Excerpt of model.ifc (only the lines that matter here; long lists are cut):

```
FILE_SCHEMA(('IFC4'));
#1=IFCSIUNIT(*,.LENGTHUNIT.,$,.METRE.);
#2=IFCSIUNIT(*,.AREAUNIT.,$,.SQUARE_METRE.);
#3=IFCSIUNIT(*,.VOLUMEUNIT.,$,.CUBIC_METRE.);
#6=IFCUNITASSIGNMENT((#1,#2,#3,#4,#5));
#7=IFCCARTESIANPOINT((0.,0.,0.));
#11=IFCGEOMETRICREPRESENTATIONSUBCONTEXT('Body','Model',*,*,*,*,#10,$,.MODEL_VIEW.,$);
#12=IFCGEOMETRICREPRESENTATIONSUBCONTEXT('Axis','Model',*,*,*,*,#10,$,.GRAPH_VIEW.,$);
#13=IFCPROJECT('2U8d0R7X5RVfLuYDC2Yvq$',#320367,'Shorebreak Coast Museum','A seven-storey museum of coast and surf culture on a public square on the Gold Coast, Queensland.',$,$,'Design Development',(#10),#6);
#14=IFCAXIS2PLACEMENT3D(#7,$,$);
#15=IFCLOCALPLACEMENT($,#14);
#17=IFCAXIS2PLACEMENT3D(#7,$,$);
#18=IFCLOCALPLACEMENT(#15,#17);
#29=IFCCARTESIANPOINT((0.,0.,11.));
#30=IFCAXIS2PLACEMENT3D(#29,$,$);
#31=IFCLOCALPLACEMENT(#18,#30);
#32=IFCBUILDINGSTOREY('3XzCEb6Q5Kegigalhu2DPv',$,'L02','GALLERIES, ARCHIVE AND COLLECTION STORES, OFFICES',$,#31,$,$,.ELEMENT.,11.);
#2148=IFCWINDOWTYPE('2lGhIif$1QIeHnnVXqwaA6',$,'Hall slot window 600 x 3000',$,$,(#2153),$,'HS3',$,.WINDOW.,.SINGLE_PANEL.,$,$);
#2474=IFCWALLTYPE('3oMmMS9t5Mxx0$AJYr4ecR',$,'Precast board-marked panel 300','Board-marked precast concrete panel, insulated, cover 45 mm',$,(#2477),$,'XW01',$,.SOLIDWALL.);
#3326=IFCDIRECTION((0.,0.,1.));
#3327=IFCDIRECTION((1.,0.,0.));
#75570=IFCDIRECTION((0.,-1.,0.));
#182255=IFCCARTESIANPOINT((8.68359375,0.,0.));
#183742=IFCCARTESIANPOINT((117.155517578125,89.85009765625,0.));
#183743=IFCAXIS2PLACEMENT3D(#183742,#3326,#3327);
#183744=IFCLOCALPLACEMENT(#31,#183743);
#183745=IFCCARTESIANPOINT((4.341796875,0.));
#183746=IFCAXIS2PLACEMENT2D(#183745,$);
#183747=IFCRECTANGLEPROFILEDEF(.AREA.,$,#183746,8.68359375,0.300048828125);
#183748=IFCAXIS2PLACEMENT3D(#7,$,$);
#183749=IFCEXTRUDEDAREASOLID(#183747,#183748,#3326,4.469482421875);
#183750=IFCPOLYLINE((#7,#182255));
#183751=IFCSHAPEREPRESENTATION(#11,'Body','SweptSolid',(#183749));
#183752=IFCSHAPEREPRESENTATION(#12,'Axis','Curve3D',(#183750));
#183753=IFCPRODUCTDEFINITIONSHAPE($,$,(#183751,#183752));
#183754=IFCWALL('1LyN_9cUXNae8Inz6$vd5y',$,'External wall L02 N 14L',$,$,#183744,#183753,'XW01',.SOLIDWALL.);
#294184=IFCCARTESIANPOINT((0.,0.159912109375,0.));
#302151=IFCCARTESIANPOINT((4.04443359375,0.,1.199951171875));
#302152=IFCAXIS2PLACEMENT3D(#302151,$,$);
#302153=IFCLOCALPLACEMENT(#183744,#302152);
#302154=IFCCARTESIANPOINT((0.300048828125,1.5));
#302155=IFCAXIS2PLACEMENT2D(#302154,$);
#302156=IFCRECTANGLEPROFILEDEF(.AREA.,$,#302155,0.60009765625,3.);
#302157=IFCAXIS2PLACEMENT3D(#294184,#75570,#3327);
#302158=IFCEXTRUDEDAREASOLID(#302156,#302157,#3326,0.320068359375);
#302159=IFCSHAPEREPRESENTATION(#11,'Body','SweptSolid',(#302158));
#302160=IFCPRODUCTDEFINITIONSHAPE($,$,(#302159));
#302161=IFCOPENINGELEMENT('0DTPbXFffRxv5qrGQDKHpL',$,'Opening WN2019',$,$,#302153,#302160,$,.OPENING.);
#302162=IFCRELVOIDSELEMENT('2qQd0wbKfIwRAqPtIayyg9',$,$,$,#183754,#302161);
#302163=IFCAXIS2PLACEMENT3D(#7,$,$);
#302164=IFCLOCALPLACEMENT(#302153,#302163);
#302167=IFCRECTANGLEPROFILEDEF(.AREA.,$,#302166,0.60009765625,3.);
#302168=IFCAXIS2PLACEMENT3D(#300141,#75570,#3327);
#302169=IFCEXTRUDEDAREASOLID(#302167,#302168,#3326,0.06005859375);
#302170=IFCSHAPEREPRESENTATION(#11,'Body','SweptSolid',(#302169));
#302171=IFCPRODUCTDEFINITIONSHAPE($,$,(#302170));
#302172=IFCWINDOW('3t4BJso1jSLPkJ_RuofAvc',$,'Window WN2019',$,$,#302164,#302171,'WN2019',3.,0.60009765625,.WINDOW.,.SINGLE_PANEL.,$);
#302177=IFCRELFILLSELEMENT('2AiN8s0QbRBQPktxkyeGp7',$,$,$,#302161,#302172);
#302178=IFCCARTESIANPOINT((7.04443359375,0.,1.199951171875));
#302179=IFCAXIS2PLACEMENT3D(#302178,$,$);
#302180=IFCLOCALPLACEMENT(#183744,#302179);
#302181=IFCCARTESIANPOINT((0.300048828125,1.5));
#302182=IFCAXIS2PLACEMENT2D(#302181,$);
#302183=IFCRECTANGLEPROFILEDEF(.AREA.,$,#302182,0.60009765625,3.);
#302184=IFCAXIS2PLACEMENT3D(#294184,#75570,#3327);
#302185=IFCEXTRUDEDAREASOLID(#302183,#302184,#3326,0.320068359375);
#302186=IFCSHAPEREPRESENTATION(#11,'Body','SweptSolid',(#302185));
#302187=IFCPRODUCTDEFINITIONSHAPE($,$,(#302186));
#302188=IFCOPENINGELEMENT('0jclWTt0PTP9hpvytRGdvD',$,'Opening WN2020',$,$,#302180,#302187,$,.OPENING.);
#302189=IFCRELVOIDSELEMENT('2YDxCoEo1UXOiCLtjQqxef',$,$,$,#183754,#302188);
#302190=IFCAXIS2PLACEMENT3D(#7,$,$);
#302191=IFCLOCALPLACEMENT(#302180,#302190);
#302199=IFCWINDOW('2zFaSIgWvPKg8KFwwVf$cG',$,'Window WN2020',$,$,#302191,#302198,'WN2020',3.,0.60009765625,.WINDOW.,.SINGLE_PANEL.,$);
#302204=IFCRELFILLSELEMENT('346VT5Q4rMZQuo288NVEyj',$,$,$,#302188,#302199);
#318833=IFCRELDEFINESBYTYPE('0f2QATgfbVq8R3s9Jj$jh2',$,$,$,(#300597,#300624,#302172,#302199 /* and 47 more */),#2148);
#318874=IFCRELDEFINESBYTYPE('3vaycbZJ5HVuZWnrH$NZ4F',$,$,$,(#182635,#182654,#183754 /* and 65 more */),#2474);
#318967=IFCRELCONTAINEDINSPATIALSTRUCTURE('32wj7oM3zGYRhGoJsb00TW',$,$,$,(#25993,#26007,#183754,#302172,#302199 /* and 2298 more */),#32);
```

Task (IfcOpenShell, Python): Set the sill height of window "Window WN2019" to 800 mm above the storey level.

```python
import numpy as np
import ifcopenshell
import ifcopenshell.api.geometry
import ifcopenshell.geom
import ifcopenshell.util.element
import ifcopenshell.util.placement
import ifcopenshell.util.shape
import ifcopenshell.util.unit

model = ifcopenshell.open("model.ifc")
unit_scale = ifcopenshell.util.unit.calculate_unit_scale(model)

window = model.by_guid("3t4BJso1jSLPkJ_RuofAvc")
opening = window.FillsVoids[0].RelatingOpeningElement
storey = ifcopenshell.util.element.get_container(window, ifc_class="IfcBuildingStorey")
level = ifcopenshell.util.placement.get_local_placement(storey.ObjectPlacement)[2, 3]

# The opening's origin need not be at the sill, so measure its lowest point.
shape = ifcopenshell.geom.create_shape(ifcopenshell.geom.settings(), opening)
bottom = ifcopenshell.util.shape.get_shape_bottom_elevation(shape, shape.geometry) / unit_scale
dz = level + 0.8 / unit_scale - bottom

shift = np.array([0.0, 0.0, dz])
# The window is placed relative to its opening, so it follows when the opening moves.
matrix = ifcopenshell.util.placement.get_local_placement(opening.ObjectPlacement)
matrix[:3, 3] += shift
ifcopenshell.api.geometry.edit_object_placement(
    model, product=opening, matrix=matrix, is_si=False, should_transform_children=True
)

print(f"moved by {dz * unit_scale:+.3f} m")

model.write("model_rev.ifc")
```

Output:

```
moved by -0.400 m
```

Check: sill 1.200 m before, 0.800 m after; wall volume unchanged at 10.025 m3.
